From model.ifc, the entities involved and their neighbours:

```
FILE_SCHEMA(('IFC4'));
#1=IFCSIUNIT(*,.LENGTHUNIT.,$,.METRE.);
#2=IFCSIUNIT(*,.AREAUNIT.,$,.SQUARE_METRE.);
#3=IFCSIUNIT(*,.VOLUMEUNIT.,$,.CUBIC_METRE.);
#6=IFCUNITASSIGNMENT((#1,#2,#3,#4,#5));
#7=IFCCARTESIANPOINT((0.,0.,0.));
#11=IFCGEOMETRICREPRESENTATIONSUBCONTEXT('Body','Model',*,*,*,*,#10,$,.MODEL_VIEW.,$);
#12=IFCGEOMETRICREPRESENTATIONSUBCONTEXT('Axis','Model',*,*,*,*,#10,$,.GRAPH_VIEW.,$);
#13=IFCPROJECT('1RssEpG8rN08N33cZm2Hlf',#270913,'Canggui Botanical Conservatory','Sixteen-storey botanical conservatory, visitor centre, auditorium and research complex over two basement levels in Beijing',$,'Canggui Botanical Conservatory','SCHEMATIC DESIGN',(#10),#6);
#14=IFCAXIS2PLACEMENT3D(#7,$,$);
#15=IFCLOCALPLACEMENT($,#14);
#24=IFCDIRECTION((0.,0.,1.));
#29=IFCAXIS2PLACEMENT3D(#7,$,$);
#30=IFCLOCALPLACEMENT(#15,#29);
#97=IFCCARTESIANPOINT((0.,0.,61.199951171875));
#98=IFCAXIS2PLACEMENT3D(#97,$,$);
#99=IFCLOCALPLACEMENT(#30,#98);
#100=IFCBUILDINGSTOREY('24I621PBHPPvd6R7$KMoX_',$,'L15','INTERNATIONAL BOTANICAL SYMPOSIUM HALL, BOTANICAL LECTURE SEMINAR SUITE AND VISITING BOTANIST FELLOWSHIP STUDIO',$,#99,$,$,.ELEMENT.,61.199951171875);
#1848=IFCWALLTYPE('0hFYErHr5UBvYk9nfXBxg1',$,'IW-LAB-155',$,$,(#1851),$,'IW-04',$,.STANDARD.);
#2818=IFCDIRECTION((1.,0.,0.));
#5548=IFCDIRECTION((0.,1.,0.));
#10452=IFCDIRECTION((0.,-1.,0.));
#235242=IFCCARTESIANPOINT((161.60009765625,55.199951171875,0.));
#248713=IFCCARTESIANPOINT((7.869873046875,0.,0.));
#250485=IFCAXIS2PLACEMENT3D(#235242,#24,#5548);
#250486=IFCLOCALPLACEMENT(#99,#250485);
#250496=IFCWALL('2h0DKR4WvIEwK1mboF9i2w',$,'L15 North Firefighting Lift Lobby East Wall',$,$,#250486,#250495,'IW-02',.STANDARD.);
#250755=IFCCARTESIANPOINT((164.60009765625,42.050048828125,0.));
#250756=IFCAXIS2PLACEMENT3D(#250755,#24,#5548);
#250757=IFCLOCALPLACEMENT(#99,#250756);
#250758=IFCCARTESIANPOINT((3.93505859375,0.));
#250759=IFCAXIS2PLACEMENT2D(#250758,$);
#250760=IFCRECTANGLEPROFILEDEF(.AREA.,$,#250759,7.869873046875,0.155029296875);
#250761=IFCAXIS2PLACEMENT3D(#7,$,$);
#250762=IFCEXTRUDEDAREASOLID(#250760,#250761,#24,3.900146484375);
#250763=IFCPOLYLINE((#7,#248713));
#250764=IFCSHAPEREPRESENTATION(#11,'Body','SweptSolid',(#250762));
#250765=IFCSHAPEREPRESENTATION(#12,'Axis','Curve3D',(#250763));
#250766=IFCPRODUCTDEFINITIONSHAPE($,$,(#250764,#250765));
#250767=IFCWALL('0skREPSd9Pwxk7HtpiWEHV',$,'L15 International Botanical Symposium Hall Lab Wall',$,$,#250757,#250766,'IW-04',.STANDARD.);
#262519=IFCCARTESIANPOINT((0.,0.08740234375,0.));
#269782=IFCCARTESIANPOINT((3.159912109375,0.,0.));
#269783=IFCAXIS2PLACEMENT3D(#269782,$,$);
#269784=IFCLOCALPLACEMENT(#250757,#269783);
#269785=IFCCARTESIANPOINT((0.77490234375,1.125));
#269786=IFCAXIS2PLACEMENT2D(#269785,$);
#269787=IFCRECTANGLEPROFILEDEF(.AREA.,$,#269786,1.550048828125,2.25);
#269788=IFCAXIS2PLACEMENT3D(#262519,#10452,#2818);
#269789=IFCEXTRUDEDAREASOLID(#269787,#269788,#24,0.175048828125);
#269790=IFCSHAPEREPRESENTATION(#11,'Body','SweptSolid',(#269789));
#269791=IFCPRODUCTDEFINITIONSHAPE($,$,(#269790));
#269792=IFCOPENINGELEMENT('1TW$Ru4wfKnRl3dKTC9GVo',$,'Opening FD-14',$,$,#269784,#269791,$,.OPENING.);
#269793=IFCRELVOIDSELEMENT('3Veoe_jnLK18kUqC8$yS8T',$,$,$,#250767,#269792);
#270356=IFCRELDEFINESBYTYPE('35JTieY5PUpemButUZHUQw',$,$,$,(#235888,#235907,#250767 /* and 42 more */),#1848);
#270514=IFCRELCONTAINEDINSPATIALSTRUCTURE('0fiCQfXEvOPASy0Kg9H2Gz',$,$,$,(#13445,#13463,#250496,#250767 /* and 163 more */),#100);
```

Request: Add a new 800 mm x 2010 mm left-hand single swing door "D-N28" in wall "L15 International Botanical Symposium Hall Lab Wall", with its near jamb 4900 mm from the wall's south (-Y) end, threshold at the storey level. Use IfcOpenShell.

```python
import numpy as np
import ifcopenshell
import ifcopenshell.api.feature
import ifcopenshell.api.geometry
import ifcopenshell.api.root
import ifcopenshell.api.spatial
import ifcopenshell.geom
import ifcopenshell.util.element
import ifcopenshell.util.placement
import ifcopenshell.util.representation
import ifcopenshell.util.shape
import ifcopenshell.util.unit

model = ifcopenshell.open("model.ifc")
unit_scale = ifcopenshell.util.unit.calculate_unit_scale(model)
settings = ifcopenshell.geom.settings()


def volume(element):
    """Net volume in cubic metres, openings subtracted."""
    shape = ifcopenshell.geom.create_shape(settings, element)
    return ifcopenshell.util.shape.get_volume(shape.geometry)


wall = model.by_id(250767)
storey = ifcopenshell.util.element.get_container(wall, ifc_class="IfcBuildingStorey")
context = ifcopenshell.util.representation.get_context(model, "Model", "Body", "MODEL_VIEW")
before = volume(wall)

width, height, from_end, sill = 0.8, 2.01, 4.9, 0.0  # metres

# The wall runs along its own X axis, and the end named is its -X end.
wall_shape = ifcopenshell.geom.create_shape(settings, wall)
x, y, z = ifcopenshell.util.shape.get_vertices(wall_shape.geometry).T
start = x.min() + from_end
face, thickness = float(y.min()), float(y.max() - y.min())
wall_matrix = ifcopenshell.util.placement.get_local_placement(wall.ObjectPlacement)
level = ifcopenshell.util.placement.get_local_placement(storey.ObjectPlacement)[2, 3]


def in_wall(x, y):
    """Placement at x, y metres in the wall's axes, at sill height."""
    matrix = wall_matrix.copy()
    matrix[:, 3] = wall_matrix @ np.array([x / unit_scale, y / unit_scale, 0.0, 1.0])
    matrix[2, 3] = level + sill / unit_scale
    return matrix


# Opening: a box that overshoots both wall faces by 50 mm.
opening = ifcopenshell.api.root.create_entity(model, ifc_class="IfcOpeningElement", predefined_type="OPENING")
box = ifcopenshell.api.geometry.add_wall_representation(
    model, context=context, length=width, height=height, thickness=thickness + 0.1
)
ifcopenshell.api.geometry.assign_representation(model, product=opening, representation=box)
ifcopenshell.api.geometry.edit_object_placement(model, product=opening, matrix=in_wall(start, face - 0.05), is_si=False)
ifcopenshell.api.feature.add_feature(model, feature=opening, element=wall)

door = ifcopenshell.api.root.create_entity(model, ifc_class="IfcDoor", name="D-N28", predefined_type="DOOR")
door.OverallWidth, door.OverallHeight = width / unit_scale, height / unit_scale
door.OperationType = "SINGLE_SWING_LEFT"
body = ifcopenshell.api.geometry.add_door_representation(
    model,
    context=context,
    overall_width=door.OverallWidth,
    overall_height=door.OverallHeight,
    operation_type="SINGLE_SWING_LEFT",
    lining_properties={"LiningDepth": thickness / unit_scale, "ThresholdDepth": thickness / unit_scale},
)
ifcopenshell.api.geometry.assign_representation(model, product=door, representation=body)
ifcopenshell.api.spatial.assign_container(model, products=[door], relating_structure=storey)
ifcopenshell.api.feature.add_filling(model, opening=opening, element=door)

# The lining spans the wall, so the door starts at the wall face.
ifcopenshell.api.geometry.edit_object_placement(model, product=door, matrix=in_wall(start, face), is_si=False)

after = volume(wall)

print(f"wall volume {before:.3f} -> {after:.3f} m3")

model.write("model_edited.ifc")
```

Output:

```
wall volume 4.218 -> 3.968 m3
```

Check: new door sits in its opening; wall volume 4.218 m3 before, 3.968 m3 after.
